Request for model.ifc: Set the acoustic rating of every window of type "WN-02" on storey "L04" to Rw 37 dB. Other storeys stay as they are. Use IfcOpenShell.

First a look at what the model holds.

```python
import ifcopenshell
import ifcopenshell.util.element

model = ifcopenshell.open("model.ifc")
print(model.schema)
storey = next(s for s in model.by_type("IfcBuildingStorey") if s.Name == "L04")
windows = [e for e in ifcopenshell.util.element.get_decomposition(storey) if e.is_a("IfcWindow")]
seen = {}
for e in windows:
    element_type = ifcopenshell.util.element.get_type(e)
    key = (element_type.Name if element_type != e and element_type else None, ifcopenshell.util.element.get_pset(e, "Pset_WindowCommon", "AcousticRating"))
    seen[key] = seen.get(key, 0) + 1
for (name, value), count in sorted(seen.items(), key=str):
    print(count, "x", name, "|", value)
```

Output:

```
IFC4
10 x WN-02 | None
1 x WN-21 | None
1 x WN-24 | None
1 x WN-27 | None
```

```python
import ifcopenshell
import ifcopenshell.api.pset
import ifcopenshell.util.element

model = ifcopenshell.open("model.ifc")

storey = next(s for s in model.by_type("IfcBuildingStorey") if s.Name == "L04")
windows = [e for e in ifcopenshell.util.element.get_decomposition(storey) if e.is_a("IfcWindow")]

count = 0
for e in windows:
    element_type = ifcopenshell.util.element.get_type(e)
    if element_type in (None, e) or element_type.Name != "WN-02":
        continue
    # add_pset returns the element's existing set when there is one.
    pset = ifcopenshell.api.pset.add_pset(model, product=e, name="Pset_WindowCommon")
    ifcopenshell.api.pset.edit_pset(model, pset=pset, properties={"AcousticRating": "Rw 37 dB"})
    count += 1

print(count, "windows updated")

model.write("model-out.ifc")
```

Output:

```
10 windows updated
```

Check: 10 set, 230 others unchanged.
